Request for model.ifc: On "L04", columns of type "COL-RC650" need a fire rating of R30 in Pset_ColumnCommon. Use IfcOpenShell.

First a look at what the model holds.

```python
import ifcopenshell
import ifcopenshell.util.element

model = ifcopenshell.open("model.ifc")
print(model.schema)
storey = next(s for s in model.by_type("IfcBuildingStorey") if s.Name == "L04")
columns = [e for e in ifcopenshell.util.element.get_decomposition(storey) if e.is_a("IfcColumn")]
seen = {}
for e in columns:
    element_type = ifcopenshell.util.element.get_type(e)
    key = (element_type.Name if element_type != e and element_type else None, ifcopenshell.util.element.get_pset(e, "Pset_ColumnCommon", "FireRating"))
    seen[key] = seen.get(key, 0) + 1
for (name, value), count in sorted(seen.items(), key=str):
    print(count, "x", name, "|", value)
```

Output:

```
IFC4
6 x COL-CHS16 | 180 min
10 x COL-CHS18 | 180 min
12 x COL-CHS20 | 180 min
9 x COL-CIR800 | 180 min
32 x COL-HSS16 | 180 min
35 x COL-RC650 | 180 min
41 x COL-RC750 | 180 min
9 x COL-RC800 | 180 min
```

```python
import ifcopenshell
import ifcopenshell.api.pset
import ifcopenshell.util.element

model = ifcopenshell.open("model.ifc")

storey = next(s for s in model.by_type("IfcBuildingStorey") if s.Name == "L04")
columns = [e for e in ifcopenshell.util.element.get_decomposition(storey) if e.is_a("IfcColumn")]

count = 0
for e in columns:
    element_type = ifcopenshell.util.element.get_type(e)
    if element_type in (None, e) or element_type.Name != "COL-RC650":
        continue
    # add_pset returns the element's existing set when there is one.
    pset = ifcopenshell.api.pset.add_pset(model, product=e, name="Pset_ColumnCommon")
    ifcopenshell.api.pset.edit_pset(model, pset=pset, properties={"FireRating": "R30"})
    count += 1

print(count, "columns updated")

model.write("model_rev.ifc")
```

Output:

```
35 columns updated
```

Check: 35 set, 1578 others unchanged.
